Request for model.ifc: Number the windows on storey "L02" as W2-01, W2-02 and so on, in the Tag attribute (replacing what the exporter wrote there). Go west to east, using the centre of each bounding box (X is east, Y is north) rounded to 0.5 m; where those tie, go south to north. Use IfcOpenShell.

First a look at what the model holds.

```python
import ifcopenshell
import ifcopenshell.util.element
import ifcopenshell.util.placement

model = ifcopenshell.open("model.ifc")
print(model.schema)
storey = next(s for s in model.by_type("IfcBuildingStorey") if s.Name == "L02")
windows = [e for e in ifcopenshell.util.element.get_decomposition(storey) if e.is_a("IfcWindow")]
for e in sorted(windows, key=lambda e: e.id()):
    origin = ifcopenshell.util.placement.get_local_placement(e.ObjectPlacement)[:3, 3]
    print(e.id(), e.Tag, e.Name, origin.round(2) + 0.0, sep=" | ")
```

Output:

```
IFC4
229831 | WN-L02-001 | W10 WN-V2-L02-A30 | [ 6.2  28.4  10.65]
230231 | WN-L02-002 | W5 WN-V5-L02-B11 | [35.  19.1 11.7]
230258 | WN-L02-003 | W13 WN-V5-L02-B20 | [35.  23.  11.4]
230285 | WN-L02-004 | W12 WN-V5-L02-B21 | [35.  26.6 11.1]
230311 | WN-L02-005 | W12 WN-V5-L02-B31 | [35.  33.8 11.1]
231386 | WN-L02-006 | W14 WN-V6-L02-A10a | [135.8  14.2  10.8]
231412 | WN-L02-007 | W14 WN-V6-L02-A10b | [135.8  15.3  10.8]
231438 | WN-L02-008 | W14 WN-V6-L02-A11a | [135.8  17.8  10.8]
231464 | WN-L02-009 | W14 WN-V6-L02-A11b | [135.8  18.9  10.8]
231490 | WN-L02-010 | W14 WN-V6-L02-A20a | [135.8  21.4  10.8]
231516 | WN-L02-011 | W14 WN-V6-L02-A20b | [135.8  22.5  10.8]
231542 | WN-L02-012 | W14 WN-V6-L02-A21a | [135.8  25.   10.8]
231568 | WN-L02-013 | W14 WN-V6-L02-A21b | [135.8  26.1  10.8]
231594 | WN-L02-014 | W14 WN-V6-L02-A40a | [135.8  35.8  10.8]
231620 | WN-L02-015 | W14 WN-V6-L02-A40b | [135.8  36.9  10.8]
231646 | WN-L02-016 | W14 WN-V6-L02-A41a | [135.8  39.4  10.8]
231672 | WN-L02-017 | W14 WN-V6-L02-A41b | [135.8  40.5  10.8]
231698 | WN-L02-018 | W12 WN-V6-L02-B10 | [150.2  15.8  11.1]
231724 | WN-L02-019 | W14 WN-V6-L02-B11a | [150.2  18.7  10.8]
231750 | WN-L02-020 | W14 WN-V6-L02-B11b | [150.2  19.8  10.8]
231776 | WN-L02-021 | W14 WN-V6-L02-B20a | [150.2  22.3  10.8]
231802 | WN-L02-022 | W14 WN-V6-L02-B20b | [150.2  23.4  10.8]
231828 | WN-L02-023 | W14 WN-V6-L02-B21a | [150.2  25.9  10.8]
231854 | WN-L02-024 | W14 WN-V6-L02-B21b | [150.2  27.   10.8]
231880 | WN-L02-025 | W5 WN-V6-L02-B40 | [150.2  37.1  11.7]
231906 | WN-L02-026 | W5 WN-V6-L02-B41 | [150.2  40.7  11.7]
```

```python
import ifcopenshell
import ifcopenshell.geom
import ifcopenshell.util.element
import ifcopenshell.util.shape

model = ifcopenshell.open("model.ifc")
settings = ifcopenshell.geom.settings()
settings.set("use-world-coords", True)


def centre(element):
    shape = ifcopenshell.geom.create_shape(settings, element)
    return ifcopenshell.util.shape.get_bbox_centroid(shape.geometry)


storey = next(s for s in model.by_type("IfcBuildingStorey") if s.Name == "L02")
windows = [e for e in ifcopenshell.util.element.get_decomposition(storey) if e.is_a("IfcWindow")]

# Insertion points can sit at a corner or the storey origin, so sort by the geometry (in metres).
centres = {e: centre(e) for e in windows}
windows.sort(key=lambda e: (round(centres[e][0] / 0.5), centres[e][1]))

for i, e in enumerate(windows, start=1):
    number = f"W2-{i:02d}"
    e.Tag = number
    print(e.id(), number)

model.write("model_updated.ifc")
```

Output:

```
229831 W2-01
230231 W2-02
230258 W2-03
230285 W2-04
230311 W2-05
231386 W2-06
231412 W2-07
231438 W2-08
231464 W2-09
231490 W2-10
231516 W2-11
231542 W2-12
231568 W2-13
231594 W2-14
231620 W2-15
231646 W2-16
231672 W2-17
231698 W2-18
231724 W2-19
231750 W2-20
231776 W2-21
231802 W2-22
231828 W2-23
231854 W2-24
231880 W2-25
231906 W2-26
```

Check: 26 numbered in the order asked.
